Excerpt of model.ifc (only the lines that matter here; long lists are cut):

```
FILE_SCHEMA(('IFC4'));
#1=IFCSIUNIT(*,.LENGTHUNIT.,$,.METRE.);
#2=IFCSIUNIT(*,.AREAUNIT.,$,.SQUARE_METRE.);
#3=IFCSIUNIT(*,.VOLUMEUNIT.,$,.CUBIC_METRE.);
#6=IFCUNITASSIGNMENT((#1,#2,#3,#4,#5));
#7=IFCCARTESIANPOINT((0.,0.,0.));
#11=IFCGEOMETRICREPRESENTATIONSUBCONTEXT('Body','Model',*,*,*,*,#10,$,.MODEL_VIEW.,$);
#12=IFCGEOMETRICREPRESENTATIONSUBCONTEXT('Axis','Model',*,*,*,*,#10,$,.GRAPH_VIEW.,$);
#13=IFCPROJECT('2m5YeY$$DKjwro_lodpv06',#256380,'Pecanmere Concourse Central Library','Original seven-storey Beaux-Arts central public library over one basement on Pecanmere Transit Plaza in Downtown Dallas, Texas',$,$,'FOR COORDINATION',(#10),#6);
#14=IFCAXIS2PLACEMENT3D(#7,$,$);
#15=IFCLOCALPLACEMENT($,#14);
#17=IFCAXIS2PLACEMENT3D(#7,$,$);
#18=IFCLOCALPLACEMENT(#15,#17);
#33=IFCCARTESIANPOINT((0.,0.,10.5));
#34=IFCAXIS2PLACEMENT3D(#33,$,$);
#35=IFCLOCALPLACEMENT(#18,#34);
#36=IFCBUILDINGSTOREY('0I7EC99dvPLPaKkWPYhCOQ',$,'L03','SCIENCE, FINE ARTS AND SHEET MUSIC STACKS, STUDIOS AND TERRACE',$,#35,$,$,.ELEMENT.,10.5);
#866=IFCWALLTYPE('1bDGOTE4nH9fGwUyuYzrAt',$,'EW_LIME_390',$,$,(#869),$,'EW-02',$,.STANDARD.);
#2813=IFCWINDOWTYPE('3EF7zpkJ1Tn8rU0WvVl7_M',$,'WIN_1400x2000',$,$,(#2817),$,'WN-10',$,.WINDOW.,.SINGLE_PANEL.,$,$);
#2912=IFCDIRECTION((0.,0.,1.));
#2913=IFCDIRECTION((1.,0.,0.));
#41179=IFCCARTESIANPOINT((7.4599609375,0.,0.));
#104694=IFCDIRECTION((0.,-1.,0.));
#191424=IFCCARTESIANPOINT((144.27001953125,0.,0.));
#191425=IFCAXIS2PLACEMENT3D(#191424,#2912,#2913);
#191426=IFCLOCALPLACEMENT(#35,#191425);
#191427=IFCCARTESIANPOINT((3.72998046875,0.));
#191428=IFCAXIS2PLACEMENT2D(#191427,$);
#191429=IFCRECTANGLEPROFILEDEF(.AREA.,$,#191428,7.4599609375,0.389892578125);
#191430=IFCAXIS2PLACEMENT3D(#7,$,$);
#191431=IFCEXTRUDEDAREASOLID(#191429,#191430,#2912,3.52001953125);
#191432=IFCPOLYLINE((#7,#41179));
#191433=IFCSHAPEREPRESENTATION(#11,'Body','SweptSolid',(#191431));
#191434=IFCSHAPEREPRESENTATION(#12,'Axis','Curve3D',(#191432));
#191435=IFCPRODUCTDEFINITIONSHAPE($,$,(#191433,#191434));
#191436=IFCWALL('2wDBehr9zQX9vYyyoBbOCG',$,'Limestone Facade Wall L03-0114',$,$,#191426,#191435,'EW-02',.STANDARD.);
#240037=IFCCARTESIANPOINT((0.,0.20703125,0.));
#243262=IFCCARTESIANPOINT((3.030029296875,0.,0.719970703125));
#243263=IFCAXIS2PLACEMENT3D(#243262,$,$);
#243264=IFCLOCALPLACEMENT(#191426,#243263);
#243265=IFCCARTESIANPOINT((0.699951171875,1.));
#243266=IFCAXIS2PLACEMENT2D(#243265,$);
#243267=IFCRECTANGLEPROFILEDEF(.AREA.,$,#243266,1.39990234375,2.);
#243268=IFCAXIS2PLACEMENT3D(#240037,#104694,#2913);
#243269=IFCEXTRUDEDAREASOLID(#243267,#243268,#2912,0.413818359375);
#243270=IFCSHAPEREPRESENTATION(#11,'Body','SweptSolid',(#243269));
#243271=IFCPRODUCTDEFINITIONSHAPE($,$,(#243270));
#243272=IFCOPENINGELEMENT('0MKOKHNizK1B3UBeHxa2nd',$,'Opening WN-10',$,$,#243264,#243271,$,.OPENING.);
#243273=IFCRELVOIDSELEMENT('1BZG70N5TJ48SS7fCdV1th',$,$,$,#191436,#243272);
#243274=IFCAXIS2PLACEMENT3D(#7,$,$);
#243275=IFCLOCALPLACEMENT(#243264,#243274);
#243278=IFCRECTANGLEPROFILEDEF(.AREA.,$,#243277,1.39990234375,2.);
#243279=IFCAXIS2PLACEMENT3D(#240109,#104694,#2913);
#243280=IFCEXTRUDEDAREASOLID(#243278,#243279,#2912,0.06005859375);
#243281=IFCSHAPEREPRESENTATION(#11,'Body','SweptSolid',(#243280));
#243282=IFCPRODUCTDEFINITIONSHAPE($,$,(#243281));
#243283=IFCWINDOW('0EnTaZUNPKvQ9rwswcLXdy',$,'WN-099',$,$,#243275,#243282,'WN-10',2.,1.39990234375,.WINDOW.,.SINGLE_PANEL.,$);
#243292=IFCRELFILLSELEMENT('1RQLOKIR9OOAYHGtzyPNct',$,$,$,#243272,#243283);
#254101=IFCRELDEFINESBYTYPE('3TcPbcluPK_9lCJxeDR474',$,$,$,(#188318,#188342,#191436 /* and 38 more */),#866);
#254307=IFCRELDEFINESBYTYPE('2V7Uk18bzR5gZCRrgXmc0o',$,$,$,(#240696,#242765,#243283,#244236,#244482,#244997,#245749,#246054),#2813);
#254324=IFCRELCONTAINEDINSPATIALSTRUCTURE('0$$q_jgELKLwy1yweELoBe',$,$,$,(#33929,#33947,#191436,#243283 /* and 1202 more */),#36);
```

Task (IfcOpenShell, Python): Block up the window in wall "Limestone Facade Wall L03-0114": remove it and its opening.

```python
import ifcopenshell
import ifcopenshell.api.feature
import ifcopenshell.api.root
import ifcopenshell.geom
import ifcopenshell.util.shape

model = ifcopenshell.open("model.ifc")
settings = ifcopenshell.geom.settings()


def volume(element):
    """Net volume in cubic metres, openings subtracted."""
    shape = ifcopenshell.geom.create_shape(settings, element)
    return ifcopenshell.util.shape.get_volume(shape.geometry)


window = model.by_guid("0EnTaZUNPKvQ9rwswcLXdy")
opening = window.FillsVoids[0].RelatingOpeningElement
wall = opening.VoidsElements[0].RelatingBuildingElement
before = volume(wall)

ifcopenshell.api.root.remove_product(model, product=window)
ifcopenshell.api.feature.remove_feature(model, feature=opening)

after = volume(wall)

print(f"wall volume {before:.3f} -> {after:.3f} m3")

model.write("model-out.ifc")
```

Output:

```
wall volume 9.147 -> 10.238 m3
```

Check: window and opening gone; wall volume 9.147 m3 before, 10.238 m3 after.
